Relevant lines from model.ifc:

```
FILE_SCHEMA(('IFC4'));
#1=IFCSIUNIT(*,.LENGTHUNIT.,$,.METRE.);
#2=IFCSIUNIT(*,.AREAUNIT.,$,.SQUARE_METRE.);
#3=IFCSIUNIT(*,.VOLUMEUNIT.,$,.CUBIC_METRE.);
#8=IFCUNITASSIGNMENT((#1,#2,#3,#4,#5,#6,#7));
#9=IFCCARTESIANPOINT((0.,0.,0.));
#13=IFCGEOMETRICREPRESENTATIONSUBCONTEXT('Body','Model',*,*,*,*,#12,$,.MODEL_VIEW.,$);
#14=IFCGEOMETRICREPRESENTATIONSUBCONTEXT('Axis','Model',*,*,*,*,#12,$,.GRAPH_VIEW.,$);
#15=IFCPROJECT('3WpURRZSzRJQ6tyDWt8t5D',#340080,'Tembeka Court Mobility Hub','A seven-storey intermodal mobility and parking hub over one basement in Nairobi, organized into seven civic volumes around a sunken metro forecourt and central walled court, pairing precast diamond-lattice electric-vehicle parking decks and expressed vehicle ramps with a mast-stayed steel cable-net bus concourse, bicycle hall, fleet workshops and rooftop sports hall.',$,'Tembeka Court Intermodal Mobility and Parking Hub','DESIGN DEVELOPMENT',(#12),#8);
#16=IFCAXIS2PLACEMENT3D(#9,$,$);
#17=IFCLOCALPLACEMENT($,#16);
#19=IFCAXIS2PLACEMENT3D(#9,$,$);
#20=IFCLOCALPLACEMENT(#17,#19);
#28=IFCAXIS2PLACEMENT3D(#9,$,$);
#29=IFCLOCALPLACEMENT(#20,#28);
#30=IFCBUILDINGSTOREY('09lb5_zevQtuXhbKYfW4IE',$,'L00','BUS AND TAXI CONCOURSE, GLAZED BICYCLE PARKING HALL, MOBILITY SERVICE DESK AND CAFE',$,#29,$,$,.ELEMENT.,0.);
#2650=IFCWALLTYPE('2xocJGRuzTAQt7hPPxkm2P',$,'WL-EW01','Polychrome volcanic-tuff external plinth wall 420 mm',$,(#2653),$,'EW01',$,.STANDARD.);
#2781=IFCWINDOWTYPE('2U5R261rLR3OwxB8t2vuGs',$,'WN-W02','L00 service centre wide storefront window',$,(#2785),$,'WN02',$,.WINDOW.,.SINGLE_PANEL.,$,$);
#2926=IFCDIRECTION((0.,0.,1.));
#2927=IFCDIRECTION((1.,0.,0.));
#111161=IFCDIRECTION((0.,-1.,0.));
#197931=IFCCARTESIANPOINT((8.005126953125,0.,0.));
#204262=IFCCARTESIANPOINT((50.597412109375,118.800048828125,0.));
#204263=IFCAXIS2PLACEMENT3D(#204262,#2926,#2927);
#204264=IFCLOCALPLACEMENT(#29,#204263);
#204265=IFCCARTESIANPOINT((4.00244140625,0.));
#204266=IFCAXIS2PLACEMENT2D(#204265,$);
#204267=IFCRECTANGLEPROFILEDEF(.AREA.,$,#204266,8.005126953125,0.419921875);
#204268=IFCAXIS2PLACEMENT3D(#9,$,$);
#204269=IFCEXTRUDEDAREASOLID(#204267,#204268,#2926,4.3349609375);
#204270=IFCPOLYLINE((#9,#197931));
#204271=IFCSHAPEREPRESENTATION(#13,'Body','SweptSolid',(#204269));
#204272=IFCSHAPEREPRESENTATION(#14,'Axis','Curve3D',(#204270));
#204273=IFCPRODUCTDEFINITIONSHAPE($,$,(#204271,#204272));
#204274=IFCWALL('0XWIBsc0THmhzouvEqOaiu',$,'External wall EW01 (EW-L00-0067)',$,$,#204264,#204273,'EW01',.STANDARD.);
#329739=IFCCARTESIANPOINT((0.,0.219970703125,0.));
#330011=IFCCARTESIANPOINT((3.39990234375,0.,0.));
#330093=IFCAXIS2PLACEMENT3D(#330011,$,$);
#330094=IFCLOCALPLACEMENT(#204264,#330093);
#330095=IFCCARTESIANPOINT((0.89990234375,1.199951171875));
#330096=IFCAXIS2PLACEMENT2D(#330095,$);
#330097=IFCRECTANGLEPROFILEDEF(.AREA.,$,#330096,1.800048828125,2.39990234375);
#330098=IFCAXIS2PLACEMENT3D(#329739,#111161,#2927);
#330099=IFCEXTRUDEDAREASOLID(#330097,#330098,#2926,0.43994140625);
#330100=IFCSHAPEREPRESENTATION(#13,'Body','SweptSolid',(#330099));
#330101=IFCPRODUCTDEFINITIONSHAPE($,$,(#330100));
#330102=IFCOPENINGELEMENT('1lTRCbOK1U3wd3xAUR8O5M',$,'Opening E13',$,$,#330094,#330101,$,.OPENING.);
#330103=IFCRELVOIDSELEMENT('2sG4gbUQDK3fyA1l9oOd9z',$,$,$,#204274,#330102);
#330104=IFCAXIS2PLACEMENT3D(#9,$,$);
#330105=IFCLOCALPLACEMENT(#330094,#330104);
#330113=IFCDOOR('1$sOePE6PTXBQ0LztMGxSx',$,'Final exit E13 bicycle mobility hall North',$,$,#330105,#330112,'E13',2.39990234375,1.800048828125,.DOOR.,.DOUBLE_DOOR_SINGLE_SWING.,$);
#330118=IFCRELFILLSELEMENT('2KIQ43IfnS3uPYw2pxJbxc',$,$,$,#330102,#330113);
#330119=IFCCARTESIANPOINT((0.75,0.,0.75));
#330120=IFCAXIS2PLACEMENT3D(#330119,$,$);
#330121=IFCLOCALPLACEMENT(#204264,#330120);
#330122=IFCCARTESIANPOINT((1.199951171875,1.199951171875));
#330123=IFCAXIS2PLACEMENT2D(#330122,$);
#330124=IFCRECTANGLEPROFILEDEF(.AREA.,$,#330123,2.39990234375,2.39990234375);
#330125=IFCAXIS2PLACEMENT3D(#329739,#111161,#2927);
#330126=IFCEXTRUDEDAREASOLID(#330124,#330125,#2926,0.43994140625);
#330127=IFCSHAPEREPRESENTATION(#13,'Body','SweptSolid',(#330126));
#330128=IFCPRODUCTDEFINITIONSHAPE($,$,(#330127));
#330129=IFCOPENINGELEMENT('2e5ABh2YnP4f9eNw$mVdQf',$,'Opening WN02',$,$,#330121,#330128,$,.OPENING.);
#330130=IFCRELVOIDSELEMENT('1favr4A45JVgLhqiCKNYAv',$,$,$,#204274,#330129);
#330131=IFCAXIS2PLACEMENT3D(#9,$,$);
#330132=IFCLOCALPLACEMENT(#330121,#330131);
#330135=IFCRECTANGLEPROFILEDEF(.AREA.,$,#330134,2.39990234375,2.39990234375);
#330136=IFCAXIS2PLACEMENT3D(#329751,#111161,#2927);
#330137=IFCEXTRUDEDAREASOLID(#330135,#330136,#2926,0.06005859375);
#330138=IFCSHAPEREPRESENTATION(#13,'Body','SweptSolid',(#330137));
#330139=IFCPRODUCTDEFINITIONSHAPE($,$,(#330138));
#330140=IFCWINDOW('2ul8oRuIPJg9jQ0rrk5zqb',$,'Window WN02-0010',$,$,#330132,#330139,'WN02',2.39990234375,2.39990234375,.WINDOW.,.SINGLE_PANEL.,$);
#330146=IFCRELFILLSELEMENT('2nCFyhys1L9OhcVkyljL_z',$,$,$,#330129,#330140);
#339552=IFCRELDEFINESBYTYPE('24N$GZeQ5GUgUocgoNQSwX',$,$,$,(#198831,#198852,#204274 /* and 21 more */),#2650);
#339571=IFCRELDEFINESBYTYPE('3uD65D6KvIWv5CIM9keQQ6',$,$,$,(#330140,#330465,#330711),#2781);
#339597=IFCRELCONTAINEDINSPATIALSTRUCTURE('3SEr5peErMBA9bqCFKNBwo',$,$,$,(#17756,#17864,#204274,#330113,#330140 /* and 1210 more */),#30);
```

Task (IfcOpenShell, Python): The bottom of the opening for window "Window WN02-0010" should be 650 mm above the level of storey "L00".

```python
import numpy as np
import ifcopenshell
import ifcopenshell.api.geometry
import ifcopenshell.geom
import ifcopenshell.util.element
import ifcopenshell.util.placement
import ifcopenshell.util.shape
import ifcopenshell.util.unit

model = ifcopenshell.open("model.ifc")
unit_scale = ifcopenshell.util.unit.calculate_unit_scale(model)

window = model.by_guid("2ul8oRuIPJg9jQ0rrk5zqb")
opening = window.FillsVoids[0].RelatingOpeningElement
storey = ifcopenshell.util.element.get_container(window, ifc_class="IfcBuildingStorey")
level = ifcopenshell.util.placement.get_local_placement(storey.ObjectPlacement)[2, 3]

# The opening's origin need not be at the sill, so measure its lowest point.
shape = ifcopenshell.geom.create_shape(ifcopenshell.geom.settings(), opening)
bottom = ifcopenshell.util.shape.get_shape_bottom_elevation(shape, shape.geometry) / unit_scale
dz = level + 0.65 - bottom

shift = np.array([0.0, 0.0, dz])
# The window is placed relative to its opening, so it follows when the opening moves.
matrix = ifcopenshell.util.placement.get_local_placement(opening.ObjectPlacement)
matrix[:3, 3] += shift
ifcopenshell.api.geometry.edit_object_placement(
    model, product=opening, matrix=matrix, is_si=False, should_transform_children=True
)

print(f"moved by {dz * unit_scale:+.3f} m")

model.write("model_rev.ifc")
```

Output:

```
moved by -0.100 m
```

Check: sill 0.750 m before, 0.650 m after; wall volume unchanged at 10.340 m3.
